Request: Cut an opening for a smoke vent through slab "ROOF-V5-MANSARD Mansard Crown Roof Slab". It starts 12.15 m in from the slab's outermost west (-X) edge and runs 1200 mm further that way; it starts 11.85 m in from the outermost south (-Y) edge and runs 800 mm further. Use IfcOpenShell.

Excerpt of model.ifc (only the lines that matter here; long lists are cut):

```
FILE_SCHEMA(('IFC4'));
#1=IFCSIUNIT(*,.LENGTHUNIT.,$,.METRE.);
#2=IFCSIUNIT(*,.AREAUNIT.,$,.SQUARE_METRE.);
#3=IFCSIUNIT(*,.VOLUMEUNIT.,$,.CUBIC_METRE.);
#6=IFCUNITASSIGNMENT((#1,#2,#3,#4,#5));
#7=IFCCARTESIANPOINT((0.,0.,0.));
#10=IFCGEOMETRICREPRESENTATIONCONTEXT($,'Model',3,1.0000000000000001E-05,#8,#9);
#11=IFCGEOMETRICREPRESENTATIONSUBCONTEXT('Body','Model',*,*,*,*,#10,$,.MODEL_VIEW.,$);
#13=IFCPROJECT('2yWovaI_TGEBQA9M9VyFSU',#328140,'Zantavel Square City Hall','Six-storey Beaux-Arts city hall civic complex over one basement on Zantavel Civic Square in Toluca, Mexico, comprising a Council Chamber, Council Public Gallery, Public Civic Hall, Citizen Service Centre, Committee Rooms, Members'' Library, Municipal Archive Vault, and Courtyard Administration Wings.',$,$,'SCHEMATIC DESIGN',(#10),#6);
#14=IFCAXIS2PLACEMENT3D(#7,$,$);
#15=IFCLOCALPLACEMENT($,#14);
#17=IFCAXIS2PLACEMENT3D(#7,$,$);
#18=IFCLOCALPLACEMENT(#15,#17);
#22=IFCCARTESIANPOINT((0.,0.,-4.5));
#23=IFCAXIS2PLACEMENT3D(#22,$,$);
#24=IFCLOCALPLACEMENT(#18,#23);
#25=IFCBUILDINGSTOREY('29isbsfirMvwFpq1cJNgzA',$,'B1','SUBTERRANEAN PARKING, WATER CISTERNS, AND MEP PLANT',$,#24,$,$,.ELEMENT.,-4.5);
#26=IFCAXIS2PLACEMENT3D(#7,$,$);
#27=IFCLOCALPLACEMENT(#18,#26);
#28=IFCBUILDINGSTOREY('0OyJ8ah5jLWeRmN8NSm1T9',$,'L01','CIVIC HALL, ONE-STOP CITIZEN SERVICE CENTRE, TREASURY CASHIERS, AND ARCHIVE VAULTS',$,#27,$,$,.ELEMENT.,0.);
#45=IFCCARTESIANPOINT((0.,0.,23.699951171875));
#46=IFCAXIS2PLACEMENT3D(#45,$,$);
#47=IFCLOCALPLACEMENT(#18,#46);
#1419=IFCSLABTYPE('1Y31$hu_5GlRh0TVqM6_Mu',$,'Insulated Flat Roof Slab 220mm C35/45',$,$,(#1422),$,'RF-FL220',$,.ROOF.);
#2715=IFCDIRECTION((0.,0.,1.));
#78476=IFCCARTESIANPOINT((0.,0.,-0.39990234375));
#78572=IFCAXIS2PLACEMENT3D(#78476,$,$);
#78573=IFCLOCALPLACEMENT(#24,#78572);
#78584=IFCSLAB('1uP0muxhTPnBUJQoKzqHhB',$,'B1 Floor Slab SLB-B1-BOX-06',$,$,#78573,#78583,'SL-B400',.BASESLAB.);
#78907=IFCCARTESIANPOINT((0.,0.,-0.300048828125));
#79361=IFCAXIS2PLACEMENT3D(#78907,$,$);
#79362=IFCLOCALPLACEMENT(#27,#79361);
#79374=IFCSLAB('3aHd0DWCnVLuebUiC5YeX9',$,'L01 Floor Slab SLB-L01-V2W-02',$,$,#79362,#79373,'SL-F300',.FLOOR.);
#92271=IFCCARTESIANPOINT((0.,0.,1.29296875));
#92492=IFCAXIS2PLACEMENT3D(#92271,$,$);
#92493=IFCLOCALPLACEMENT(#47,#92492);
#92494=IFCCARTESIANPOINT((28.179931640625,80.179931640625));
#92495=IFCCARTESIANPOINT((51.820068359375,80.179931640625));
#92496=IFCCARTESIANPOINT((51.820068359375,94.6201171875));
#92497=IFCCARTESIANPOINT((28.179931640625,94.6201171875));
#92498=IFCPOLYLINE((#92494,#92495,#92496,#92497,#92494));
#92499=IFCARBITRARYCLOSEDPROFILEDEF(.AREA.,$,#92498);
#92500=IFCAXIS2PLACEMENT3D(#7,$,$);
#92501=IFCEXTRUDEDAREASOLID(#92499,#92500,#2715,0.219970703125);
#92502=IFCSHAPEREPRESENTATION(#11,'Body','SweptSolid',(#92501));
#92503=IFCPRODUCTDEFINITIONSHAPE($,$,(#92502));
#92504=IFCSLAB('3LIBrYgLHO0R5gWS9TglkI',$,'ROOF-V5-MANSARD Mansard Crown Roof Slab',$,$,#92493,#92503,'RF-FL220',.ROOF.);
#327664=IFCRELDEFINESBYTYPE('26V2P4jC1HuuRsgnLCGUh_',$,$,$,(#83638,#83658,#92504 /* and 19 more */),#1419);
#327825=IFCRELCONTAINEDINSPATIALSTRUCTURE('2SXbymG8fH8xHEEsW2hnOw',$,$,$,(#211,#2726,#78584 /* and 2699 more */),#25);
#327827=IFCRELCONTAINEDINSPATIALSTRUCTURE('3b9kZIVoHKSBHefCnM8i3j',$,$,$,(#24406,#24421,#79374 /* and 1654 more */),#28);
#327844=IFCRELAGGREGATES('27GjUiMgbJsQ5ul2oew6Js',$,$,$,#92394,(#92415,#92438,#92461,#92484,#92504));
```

```python
import numpy as np
import ifcopenshell
import ifcopenshell.api.feature
import ifcopenshell.api.geometry
import ifcopenshell.api.root
import ifcopenshell.geom
import ifcopenshell.util.placement
import ifcopenshell.util.representation
import ifcopenshell.util.shape
import ifcopenshell.util.unit

model = ifcopenshell.open("model.ifc")
unit_scale = ifcopenshell.util.unit.calculate_unit_scale(model)
settings = ifcopenshell.geom.settings()


def volume(element):
    """Net volume in cubic metres, openings subtracted."""
    shape = ifcopenshell.geom.create_shape(settings, element)
    return ifcopenshell.util.shape.get_volume(shape.geometry)


slab = model.by_guid("3LIBrYgLHO0R5gWS9TglkI")
before = volume(slab)

# Extent in the slab's own axes, in metres. The edges named are its -X and -Y sides.
slab_shape = ifcopenshell.geom.create_shape(settings, slab)
vertices = ifcopenshell.util.shape.get_vertices(slab_shape.geometry)
x_min, y_min, bottom = vertices.min(axis=0)
top = vertices[:, 2].max()

opening = ifcopenshell.api.root.create_entity(model, ifc_class="IfcOpeningElement", name="Smoke vent opening", predefined_type="OPENING")
context = ifcopenshell.util.representation.get_context(model, "Model", "Body", "MODEL_VIEW")
width, depth = 1.2, 0.8
outline = [(0.0, 0.0), (width, 0.0), (width, depth), (0.0, depth), (0.0, 0.0)]
# Overshoot both faces by 50 mm so the cut is clean.
shape = ifcopenshell.api.geometry.add_slab_representation(
    model, context=context, depth=top - bottom + 0.1, polyline=outline
)
ifcopenshell.api.geometry.assign_representation(model, product=opening, representation=shape)

matrix = ifcopenshell.util.placement.get_local_placement(slab.ObjectPlacement)
matrix[:, 3] = matrix @ np.append(np.array([x_min + 12.15, y_min + 11.85, bottom - 0.05]) / unit_scale, 1.0)
ifcopenshell.api.geometry.edit_object_placement(model, product=opening, matrix=matrix, is_si=False)
ifcopenshell.api.feature.add_feature(model, feature=opening, element=slab)

after = volume(slab)

print(f"slab volume {before:.3f} -> {after:.3f} m3")

model.write("model_edited.ifc")
```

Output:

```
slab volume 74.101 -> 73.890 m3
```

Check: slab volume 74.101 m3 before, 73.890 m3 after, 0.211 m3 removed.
